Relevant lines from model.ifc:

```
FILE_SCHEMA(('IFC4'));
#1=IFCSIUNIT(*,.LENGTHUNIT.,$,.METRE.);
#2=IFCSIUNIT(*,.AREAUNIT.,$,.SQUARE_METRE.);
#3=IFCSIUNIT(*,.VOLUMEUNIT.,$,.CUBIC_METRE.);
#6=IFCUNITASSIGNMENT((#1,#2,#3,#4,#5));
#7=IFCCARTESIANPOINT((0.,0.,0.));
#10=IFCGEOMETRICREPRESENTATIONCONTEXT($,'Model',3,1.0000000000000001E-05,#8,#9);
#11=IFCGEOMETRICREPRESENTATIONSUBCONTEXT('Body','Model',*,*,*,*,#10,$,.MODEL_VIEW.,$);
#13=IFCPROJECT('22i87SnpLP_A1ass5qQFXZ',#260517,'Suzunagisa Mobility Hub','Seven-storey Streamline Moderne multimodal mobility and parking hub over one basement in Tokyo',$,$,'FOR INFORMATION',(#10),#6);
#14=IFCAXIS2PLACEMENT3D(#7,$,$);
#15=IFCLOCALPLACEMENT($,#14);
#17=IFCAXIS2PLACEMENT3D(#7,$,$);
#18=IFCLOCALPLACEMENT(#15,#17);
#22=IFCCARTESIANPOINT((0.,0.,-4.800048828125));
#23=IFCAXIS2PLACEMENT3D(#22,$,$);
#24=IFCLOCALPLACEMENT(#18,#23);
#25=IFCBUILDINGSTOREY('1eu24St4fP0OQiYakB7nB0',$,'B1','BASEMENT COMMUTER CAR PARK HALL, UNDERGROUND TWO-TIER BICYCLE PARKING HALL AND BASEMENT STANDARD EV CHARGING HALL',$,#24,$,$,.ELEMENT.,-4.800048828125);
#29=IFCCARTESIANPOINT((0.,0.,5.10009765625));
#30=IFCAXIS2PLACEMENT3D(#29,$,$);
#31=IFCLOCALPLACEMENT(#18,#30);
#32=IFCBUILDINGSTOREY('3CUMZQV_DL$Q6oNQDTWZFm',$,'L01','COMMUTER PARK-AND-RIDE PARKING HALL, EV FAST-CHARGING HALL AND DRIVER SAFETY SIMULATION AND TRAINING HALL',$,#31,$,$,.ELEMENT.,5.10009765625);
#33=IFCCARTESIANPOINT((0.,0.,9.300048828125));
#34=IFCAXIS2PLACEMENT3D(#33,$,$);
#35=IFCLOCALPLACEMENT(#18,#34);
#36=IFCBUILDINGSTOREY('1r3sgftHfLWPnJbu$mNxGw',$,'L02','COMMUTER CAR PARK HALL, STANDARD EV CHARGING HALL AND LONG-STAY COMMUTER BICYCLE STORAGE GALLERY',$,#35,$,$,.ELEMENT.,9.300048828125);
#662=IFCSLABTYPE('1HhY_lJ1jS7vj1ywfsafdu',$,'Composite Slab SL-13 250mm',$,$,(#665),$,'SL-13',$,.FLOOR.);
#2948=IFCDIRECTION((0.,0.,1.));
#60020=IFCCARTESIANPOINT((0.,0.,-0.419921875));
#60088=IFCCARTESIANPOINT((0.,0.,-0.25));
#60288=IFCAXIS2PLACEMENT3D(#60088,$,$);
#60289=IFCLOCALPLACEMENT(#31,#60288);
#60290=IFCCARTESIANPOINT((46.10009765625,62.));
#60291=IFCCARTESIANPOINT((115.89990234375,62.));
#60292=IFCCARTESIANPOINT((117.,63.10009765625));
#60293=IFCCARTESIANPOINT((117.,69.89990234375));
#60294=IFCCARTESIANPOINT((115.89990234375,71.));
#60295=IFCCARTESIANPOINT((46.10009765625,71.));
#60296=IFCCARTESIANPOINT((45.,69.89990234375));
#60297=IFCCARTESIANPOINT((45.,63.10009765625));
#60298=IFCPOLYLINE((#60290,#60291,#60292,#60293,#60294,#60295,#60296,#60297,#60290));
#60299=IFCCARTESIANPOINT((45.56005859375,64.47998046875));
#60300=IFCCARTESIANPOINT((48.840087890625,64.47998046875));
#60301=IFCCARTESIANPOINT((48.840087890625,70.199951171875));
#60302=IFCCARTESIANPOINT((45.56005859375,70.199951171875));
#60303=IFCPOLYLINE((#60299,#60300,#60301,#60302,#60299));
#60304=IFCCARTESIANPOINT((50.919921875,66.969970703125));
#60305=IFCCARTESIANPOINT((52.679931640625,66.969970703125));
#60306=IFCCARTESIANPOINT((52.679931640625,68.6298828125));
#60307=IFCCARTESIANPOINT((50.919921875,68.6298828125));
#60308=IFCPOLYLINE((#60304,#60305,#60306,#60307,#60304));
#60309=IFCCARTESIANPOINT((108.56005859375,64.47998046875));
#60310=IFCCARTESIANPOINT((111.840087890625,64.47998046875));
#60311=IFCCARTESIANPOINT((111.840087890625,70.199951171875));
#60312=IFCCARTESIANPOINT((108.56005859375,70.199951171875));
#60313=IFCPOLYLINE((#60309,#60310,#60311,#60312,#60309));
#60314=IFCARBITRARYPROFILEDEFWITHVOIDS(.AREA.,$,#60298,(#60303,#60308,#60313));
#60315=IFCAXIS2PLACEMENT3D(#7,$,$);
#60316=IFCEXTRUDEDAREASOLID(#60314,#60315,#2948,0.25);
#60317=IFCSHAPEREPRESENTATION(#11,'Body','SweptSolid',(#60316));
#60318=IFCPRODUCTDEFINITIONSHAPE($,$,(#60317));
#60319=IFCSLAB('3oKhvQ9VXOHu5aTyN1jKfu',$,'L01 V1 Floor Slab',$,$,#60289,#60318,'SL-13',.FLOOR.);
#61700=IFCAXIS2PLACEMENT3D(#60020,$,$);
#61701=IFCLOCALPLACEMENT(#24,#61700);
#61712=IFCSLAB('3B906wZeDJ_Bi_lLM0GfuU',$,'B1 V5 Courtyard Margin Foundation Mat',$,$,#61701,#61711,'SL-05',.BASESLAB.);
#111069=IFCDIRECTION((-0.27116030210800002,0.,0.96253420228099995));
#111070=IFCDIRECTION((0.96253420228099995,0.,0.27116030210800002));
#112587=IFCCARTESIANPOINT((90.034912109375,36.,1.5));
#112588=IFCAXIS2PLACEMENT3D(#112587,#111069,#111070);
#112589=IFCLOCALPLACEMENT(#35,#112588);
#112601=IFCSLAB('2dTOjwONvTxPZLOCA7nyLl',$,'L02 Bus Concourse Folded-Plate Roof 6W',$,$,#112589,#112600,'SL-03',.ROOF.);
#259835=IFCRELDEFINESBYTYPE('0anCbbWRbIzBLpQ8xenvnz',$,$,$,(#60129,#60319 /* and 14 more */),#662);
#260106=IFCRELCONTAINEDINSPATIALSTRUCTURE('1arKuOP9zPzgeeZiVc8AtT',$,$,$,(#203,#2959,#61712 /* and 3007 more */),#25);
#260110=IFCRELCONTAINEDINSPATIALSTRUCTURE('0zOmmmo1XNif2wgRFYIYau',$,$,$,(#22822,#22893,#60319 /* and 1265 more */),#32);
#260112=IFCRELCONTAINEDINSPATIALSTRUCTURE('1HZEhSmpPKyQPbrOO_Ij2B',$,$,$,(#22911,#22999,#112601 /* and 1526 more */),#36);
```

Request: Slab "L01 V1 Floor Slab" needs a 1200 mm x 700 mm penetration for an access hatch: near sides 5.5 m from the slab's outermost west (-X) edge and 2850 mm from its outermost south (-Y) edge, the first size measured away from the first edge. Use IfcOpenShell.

```python
import numpy as np
import ifcopenshell
import ifcopenshell.api.feature
import ifcopenshell.api.geometry
import ifcopenshell.api.root
import ifcopenshell.geom
import ifcopenshell.util.placement
import ifcopenshell.util.representation
import ifcopenshell.util.shape
import ifcopenshell.util.unit

model = ifcopenshell.open("model.ifc")
unit_scale = ifcopenshell.util.unit.calculate_unit_scale(model)
settings = ifcopenshell.geom.settings()


def volume(element):
    """Net volume in cubic metres, openings subtracted."""
    shape = ifcopenshell.geom.create_shape(settings, element)
    return ifcopenshell.util.shape.get_volume(shape.geometry)


slab = model.by_guid("3oKhvQ9VXOHu5aTyN1jKfu")
before = volume(slab)

# Extent in the slab's own axes, in metres. The edges named are its -X and -Y sides.
slab_shape = ifcopenshell.geom.create_shape(settings, slab)
vertices = ifcopenshell.util.shape.get_vertices(slab_shape.geometry)
x_min, y_min, bottom = vertices.min(axis=0)
top = vertices[:, 2].max()

opening = ifcopenshell.api.root.create_entity(model, ifc_class="IfcOpeningElement", name="Access hatch opening", predefined_type="OPENING")
context = ifcopenshell.util.representation.get_context(model, "Model", "Body", "MODEL_VIEW")
width, depth = 1.2, 0.7
outline = [(0.0, 0.0), (width, 0.0), (width, depth), (0.0, depth), (0.0, 0.0)]
# Overshoot both faces by 50 mm so the cut is clean.
shape = ifcopenshell.api.geometry.add_slab_representation(
    model, context=context, depth=top - bottom + 0.1, polyline=outline
)
ifcopenshell.api.geometry.assign_representation(model, product=opening, representation=shape)

matrix = ifcopenshell.util.placement.get_local_placement(slab.ObjectPlacement)
matrix[:, 3] = matrix @ np.append(np.array([x_min + 5.5, y_min + 2.85, bottom - 0.05]) / unit_scale, 1.0)
ifcopenshell.api.geometry.edit_object_placement(model, product=opening, matrix=matrix, is_si=False)
ifcopenshell.api.feature.add_feature(model, feature=opening, element=slab)

after = volume(slab)

print(f"slab volume {before:.3f} -> {after:.3f} m3")

model.write("model_rev.ifc")
```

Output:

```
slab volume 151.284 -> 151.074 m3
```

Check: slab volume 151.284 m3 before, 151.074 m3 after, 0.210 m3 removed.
